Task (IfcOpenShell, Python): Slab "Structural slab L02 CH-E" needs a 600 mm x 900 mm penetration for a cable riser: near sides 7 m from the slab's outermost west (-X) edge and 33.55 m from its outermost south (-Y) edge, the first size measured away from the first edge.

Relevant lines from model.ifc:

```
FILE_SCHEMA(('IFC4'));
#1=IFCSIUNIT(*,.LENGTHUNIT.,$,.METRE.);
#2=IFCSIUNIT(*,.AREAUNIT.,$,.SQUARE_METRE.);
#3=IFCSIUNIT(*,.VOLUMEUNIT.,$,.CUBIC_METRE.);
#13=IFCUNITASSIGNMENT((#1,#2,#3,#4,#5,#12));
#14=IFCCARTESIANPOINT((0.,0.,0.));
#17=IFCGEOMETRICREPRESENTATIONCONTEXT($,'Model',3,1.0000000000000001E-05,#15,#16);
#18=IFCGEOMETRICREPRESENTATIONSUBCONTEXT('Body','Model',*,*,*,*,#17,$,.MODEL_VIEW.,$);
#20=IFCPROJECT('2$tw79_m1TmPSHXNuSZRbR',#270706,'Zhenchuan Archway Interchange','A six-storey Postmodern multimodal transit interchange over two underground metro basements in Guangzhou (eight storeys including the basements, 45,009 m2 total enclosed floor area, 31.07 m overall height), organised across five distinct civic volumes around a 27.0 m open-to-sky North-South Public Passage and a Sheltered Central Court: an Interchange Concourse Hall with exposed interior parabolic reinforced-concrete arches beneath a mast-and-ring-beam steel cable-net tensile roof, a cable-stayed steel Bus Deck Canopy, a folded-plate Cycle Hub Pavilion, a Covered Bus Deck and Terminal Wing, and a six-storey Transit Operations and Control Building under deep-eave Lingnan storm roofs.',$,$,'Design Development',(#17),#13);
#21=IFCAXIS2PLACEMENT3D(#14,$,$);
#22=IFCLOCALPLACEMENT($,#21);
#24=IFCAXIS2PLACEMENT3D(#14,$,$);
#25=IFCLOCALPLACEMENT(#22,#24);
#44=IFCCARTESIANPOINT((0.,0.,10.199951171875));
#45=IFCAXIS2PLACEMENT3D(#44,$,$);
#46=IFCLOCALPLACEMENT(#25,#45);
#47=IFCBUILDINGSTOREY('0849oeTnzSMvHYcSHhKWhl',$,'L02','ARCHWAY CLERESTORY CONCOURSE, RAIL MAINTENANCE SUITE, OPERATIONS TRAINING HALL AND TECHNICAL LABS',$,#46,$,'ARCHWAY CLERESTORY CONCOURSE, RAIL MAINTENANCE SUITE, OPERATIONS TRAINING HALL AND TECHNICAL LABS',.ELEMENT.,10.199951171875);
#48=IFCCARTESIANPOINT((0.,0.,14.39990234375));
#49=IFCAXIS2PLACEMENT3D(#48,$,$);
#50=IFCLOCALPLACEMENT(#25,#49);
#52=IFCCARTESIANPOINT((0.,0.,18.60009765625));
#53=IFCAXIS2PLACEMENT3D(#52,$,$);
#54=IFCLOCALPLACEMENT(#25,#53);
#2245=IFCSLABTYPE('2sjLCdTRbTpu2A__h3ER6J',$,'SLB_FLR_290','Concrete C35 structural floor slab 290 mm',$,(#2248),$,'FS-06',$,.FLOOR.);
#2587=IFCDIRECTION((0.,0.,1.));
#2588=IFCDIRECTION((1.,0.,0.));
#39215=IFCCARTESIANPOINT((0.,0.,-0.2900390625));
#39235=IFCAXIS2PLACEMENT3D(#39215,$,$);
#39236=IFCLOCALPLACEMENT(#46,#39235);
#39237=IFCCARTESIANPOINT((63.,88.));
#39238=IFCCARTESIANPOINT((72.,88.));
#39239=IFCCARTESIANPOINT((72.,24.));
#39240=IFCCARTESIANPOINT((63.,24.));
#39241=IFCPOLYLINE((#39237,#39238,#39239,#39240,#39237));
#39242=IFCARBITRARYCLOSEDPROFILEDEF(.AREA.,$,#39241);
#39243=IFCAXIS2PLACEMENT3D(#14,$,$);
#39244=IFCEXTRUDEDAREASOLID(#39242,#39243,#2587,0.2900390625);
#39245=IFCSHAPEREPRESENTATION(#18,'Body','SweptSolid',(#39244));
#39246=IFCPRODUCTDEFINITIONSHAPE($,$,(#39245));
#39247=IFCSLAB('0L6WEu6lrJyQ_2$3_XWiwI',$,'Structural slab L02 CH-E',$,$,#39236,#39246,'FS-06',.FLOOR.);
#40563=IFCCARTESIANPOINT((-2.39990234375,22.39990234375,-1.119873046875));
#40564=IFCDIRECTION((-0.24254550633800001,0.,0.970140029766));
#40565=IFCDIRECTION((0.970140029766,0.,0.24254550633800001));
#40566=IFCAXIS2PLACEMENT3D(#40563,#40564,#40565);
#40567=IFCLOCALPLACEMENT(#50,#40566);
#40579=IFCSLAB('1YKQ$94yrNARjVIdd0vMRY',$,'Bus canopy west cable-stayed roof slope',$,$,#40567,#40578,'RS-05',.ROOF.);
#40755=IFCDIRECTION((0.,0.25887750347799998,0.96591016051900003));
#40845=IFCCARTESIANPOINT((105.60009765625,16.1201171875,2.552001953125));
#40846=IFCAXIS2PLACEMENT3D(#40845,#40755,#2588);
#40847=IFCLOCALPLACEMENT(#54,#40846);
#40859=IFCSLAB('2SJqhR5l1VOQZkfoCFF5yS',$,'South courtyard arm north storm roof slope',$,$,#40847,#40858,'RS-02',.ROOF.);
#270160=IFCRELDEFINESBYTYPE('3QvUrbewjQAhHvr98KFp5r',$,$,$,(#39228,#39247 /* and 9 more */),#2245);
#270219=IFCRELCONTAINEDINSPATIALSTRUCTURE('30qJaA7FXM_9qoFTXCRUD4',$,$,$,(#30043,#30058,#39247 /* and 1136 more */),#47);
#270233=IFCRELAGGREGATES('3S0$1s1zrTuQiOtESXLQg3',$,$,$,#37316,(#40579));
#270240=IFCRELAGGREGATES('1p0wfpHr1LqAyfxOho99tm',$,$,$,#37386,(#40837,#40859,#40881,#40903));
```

```python
import numpy as np
import ifcopenshell
import ifcopenshell.api.feature
import ifcopenshell.api.geometry
import ifcopenshell.api.root
import ifcopenshell.geom
import ifcopenshell.util.placement
import ifcopenshell.util.representation
import ifcopenshell.util.shape
import ifcopenshell.util.unit

model = ifcopenshell.open("model.ifc")
unit_scale = ifcopenshell.util.unit.calculate_unit_scale(model)
settings = ifcopenshell.geom.settings()


def volume(element):
    """Net volume in cubic metres, openings subtracted."""
    shape = ifcopenshell.geom.create_shape(settings, element)
    return ifcopenshell.util.shape.get_volume(shape.geometry)


slab = model.by_guid("0L6WEu6lrJyQ_2$3_XWiwI")
before = volume(slab)

# Extent in the slab's own axes, in metres. The edges named are its -X and -Y sides.
slab_shape = ifcopenshell.geom.create_shape(settings, slab)
vertices = ifcopenshell.util.shape.get_vertices(slab_shape.geometry)
x_min, y_min, bottom = vertices.min(axis=0)
top = vertices[:, 2].max()

opening = ifcopenshell.api.root.create_entity(model, ifc_class="IfcOpeningElement", name="Cable riser opening", predefined_type="OPENING")
context = ifcopenshell.util.representation.get_context(model, "Model", "Body", "MODEL_VIEW")
width, depth = 0.6, 0.9
outline = [(0.0, 0.0), (width, 0.0), (width, depth), (0.0, depth), (0.0, 0.0)]
# Overshoot both faces by 50 mm so the cut is clean.
shape = ifcopenshell.api.geometry.add_slab_representation(
    model, context=context, depth=top - bottom + 0.1, polyline=outline
)
ifcopenshell.api.geometry.assign_representation(model, product=opening, representation=shape)

matrix = ifcopenshell.util.placement.get_local_placement(slab.ObjectPlacement)
matrix[:, 3] = matrix @ np.append(np.array([x_min + 7, y_min + 33.55, bottom - 0.05]) / unit_scale, 1.0)
ifcopenshell.api.geometry.edit_object_placement(model, product=opening, matrix=matrix, is_si=False)
ifcopenshell.api.feature.add_feature(model, feature=opening, element=slab)

after = volume(slab)

print(f"slab volume {before:.3f} -> {after:.3f} m3")

model.write("model_rev.ifc")
```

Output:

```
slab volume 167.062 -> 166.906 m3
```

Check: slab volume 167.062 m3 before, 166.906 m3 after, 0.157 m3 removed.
